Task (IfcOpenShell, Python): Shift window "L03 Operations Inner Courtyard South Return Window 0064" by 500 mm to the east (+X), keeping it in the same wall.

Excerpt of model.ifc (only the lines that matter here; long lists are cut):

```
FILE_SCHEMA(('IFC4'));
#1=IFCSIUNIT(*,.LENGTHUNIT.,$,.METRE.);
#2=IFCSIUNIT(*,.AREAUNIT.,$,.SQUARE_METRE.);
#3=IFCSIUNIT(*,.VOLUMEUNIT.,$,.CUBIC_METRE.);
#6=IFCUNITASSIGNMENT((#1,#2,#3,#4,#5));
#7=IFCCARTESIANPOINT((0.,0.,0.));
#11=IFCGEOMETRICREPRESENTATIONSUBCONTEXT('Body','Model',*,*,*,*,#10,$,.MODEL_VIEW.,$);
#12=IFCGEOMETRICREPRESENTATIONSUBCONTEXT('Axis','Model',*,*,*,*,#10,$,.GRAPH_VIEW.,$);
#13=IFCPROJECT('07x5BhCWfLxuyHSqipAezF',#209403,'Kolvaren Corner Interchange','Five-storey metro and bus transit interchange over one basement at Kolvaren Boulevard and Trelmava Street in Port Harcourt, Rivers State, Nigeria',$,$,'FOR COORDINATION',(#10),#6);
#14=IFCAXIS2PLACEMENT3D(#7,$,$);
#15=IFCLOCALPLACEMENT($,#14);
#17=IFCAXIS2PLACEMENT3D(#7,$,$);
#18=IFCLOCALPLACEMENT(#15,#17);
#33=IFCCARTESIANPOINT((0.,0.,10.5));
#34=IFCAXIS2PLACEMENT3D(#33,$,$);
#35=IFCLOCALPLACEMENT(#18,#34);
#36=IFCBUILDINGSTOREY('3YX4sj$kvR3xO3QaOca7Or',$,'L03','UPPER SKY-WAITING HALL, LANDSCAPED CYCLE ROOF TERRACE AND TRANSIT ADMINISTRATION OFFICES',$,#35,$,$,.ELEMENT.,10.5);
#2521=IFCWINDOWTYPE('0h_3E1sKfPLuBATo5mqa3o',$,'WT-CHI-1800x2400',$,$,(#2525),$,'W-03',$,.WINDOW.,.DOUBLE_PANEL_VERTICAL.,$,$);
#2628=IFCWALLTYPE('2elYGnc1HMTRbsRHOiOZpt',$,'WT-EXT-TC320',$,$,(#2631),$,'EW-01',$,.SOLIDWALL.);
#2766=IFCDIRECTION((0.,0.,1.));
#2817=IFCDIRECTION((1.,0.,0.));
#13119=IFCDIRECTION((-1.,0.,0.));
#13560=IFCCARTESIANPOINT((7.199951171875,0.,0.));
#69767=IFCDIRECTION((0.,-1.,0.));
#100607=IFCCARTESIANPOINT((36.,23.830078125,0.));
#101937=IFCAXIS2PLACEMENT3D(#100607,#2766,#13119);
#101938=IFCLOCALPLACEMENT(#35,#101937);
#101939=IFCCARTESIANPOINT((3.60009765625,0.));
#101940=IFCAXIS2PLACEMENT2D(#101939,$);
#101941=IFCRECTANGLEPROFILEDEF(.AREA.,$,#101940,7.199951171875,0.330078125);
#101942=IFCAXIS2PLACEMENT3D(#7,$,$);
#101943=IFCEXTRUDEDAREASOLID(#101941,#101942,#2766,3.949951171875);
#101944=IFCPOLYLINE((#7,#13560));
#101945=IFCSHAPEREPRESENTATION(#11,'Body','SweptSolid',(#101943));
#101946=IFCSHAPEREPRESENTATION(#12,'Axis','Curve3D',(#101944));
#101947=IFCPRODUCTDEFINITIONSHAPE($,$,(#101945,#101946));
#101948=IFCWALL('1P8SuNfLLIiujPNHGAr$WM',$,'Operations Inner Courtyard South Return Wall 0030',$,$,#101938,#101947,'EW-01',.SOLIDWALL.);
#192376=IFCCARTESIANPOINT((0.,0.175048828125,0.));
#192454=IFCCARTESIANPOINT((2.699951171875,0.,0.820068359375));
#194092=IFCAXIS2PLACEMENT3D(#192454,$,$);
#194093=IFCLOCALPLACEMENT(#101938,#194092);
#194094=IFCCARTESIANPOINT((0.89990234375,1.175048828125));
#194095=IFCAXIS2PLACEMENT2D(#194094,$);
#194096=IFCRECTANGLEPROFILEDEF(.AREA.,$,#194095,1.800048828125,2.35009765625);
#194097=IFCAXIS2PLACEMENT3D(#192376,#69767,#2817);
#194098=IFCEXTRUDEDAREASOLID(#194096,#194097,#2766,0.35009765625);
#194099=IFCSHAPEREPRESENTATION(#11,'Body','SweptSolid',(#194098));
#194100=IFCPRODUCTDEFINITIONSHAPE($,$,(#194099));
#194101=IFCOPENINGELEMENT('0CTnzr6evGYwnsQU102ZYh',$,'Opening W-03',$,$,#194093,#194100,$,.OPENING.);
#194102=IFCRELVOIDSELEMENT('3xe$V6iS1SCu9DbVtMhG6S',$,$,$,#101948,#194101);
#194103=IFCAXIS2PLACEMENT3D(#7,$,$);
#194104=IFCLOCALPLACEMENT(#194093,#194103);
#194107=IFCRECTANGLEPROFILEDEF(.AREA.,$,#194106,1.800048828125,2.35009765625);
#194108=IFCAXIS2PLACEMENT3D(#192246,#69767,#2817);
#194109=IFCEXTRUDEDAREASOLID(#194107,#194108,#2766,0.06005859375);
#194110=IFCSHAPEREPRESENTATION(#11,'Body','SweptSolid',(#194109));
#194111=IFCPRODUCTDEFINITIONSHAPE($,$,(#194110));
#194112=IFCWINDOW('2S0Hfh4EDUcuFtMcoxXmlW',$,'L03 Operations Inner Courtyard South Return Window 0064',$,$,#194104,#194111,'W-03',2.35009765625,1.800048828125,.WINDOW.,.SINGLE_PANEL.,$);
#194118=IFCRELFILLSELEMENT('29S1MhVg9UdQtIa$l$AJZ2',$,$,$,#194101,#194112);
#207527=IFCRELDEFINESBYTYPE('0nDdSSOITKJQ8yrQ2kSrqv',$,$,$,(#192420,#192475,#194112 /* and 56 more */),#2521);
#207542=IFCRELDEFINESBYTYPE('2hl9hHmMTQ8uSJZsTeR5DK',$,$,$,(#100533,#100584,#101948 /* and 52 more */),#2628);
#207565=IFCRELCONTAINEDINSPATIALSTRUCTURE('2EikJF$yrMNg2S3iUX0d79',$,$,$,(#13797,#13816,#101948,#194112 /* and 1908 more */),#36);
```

```python
import ifcopenshell
import ifcopenshell.api.geometry
import ifcopenshell.util.placement
import ifcopenshell.util.unit

model = ifcopenshell.open("model.ifc")
unit_scale = ifcopenshell.util.unit.calculate_unit_scale(model)

window = model.by_guid("2S0Hfh4EDUcuFtMcoxXmlW")
opening = window.FillsVoids[0].RelatingOpeningElement
wall = opening.VoidsElements[0].RelatingBuildingElement

wall_matrix = ifcopenshell.util.placement.get_local_placement(wall.ObjectPlacement)
shift = wall_matrix[:3, 0] * -0.5 / unit_scale
before = ifcopenshell.util.placement.get_local_placement(window.ObjectPlacement)[:3, 3].copy()

# The window is placed relative to its opening, so it follows when the opening moves.
matrix = ifcopenshell.util.placement.get_local_placement(opening.ObjectPlacement)
matrix[:3, 3] += shift
ifcopenshell.api.geometry.edit_object_placement(
    model, product=opening, matrix=matrix, is_si=False, should_transform_children=True
)

after = ifcopenshell.util.placement.get_local_placement(window.ObjectPlacement)[:3, 3]
print("window moved by", (after - before).round(3) + 0.0)

model.write("model-out.ifc")
```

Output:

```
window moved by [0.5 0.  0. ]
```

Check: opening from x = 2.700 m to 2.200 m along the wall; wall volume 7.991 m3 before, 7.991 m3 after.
